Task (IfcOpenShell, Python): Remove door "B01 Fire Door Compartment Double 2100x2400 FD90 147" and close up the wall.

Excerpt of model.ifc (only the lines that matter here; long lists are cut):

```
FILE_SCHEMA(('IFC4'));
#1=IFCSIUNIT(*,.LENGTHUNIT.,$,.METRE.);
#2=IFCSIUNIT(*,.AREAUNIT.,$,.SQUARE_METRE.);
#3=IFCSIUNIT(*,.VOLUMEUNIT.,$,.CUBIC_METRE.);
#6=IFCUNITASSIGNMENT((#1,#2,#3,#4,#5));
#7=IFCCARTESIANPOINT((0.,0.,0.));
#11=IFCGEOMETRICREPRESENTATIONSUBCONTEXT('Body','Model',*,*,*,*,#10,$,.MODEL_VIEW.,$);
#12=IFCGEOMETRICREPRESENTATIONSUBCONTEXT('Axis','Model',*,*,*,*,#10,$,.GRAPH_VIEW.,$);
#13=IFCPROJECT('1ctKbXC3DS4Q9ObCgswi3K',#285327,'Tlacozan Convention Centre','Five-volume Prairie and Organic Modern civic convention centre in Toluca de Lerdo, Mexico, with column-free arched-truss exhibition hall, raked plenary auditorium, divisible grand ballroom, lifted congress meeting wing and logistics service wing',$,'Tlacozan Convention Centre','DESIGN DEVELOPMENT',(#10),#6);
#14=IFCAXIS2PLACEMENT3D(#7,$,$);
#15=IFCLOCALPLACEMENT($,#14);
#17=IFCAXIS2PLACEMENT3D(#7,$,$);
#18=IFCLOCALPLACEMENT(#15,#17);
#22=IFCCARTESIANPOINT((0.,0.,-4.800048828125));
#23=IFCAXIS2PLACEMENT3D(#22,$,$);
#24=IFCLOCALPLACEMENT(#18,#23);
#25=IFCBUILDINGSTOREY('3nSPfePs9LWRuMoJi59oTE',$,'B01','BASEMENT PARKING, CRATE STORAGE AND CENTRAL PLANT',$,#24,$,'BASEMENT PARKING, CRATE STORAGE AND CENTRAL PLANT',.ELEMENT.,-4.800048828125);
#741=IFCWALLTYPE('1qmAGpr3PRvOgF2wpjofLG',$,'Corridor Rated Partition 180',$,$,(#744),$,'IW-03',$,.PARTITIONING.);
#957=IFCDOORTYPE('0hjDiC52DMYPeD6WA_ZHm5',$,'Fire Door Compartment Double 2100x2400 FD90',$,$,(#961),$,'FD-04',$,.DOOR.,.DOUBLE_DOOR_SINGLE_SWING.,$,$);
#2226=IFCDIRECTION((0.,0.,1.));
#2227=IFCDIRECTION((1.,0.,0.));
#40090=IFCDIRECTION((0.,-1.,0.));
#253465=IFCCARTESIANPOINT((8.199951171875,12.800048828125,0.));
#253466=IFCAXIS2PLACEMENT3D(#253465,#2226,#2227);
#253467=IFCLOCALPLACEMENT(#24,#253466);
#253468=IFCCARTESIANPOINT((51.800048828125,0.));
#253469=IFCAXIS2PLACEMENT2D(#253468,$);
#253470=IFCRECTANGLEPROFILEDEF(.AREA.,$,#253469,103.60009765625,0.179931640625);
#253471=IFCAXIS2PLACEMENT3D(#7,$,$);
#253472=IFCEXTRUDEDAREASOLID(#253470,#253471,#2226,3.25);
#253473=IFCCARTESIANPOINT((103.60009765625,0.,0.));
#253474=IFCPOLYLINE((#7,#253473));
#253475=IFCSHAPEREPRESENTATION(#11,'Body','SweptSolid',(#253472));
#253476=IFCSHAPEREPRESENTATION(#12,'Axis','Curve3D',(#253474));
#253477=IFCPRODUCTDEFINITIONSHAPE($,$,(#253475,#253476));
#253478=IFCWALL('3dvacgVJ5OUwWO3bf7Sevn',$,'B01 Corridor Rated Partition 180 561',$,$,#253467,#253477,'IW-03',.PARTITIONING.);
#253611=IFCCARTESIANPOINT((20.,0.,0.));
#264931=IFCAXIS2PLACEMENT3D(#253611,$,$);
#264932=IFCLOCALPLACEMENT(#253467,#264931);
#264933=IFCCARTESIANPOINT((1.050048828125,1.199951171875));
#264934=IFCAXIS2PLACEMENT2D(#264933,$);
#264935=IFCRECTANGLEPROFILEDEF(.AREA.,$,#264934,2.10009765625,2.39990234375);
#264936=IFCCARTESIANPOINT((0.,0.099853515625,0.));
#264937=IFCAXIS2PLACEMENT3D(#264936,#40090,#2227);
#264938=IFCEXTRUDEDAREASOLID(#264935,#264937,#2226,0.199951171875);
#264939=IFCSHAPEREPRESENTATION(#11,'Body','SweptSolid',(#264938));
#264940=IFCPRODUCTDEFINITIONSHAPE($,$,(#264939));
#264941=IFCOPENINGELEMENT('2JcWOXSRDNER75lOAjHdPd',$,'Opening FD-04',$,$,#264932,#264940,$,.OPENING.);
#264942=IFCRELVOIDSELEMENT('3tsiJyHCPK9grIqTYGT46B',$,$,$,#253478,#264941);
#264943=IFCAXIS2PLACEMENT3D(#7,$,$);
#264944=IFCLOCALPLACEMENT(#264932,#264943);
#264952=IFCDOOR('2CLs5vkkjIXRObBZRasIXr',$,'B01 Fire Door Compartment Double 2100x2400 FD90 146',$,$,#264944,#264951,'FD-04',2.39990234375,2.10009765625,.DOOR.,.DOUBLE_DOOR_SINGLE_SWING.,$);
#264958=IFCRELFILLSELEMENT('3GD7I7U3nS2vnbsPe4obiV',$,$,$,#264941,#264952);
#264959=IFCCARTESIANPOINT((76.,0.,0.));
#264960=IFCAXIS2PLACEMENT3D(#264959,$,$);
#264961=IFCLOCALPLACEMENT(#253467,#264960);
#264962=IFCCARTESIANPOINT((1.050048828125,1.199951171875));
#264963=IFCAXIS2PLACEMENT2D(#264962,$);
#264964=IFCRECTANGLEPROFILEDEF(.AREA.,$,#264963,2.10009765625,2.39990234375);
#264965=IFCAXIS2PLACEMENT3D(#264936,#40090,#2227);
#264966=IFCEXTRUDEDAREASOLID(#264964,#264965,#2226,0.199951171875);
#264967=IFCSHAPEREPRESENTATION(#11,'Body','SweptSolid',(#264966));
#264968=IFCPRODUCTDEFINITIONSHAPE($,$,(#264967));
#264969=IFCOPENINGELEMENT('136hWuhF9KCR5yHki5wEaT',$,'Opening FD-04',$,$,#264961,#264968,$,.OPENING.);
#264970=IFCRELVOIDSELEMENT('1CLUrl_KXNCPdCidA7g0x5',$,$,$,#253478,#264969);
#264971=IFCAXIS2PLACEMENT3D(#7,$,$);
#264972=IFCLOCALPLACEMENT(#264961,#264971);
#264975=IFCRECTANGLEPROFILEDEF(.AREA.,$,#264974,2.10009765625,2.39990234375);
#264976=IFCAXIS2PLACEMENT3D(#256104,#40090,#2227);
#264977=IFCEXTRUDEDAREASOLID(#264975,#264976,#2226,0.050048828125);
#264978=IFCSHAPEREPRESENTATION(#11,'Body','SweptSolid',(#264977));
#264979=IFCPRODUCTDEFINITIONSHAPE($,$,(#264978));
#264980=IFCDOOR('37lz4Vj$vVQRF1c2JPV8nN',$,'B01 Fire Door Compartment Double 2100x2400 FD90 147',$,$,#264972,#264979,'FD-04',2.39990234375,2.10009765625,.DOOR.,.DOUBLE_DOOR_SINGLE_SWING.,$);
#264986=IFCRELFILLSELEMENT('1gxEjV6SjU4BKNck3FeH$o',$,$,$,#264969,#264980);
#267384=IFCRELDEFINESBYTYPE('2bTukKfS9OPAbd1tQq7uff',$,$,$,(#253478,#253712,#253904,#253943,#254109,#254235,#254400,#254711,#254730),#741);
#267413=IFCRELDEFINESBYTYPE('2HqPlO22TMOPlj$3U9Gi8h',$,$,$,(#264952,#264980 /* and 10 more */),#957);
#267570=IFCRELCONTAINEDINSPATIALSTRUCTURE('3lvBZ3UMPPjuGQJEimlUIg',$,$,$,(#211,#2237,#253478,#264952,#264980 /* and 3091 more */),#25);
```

```python
import ifcopenshell
import ifcopenshell.api.feature
import ifcopenshell.api.root
import ifcopenshell.geom
import ifcopenshell.util.shape

model = ifcopenshell.open("model.ifc")
settings = ifcopenshell.geom.settings()


def volume(element):
    """Net volume in cubic metres, openings subtracted."""
    shape = ifcopenshell.geom.create_shape(settings, element)
    return ifcopenshell.util.shape.get_volume(shape.geometry)


door = model.by_guid("37lz4Vj$vVQRF1c2JPV8nN")
opening = door.FillsVoids[0].RelatingOpeningElement
wall = opening.VoidsElements[0].RelatingBuildingElement
before = volume(wall)

ifcopenshell.api.root.remove_product(model, product=door)
ifcopenshell.api.feature.remove_feature(model, feature=opening)

after = volume(wall)

print(f"wall volume {before:.3f} -> {after:.3f} m3")

model.write("model_edited.ifc")
```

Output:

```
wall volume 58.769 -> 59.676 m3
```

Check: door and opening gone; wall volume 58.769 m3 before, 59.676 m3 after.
